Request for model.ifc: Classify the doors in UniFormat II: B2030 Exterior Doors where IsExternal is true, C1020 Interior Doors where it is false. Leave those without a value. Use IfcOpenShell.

First a look at what the model holds.

```python
import ifcopenshell
import ifcopenshell.util.element

model = ifcopenshell.open("model.ifc")
print(model.schema)
print("classifications:", [c.Name for c in model.by_type("IfcClassification")])
values = [ifcopenshell.util.element.get_pset(e, "Pset_DoorCommon", "IsExternal") for e in model.by_type("IfcDoor")]
for value in (True, False, None):
    print("IsExternal", value, values.count(value))
```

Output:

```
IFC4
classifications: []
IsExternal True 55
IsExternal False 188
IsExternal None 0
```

```python
import ifcopenshell
import ifcopenshell.api.classification
import ifcopenshell.util.element

model = ifcopenshell.open("model.ifc")

system = ifcopenshell.api.classification.add_classification(model, classification="UniFormat II")

doors = model.by_type("IfcDoor")
external = {e: ifcopenshell.util.element.get_pset(e, "Pset_DoorCommon", "IsExternal") for e in doors}
for flag, code, name in ((True, "B2030", "Exterior Doors"), (False, "C1020", "Interior Doors")):
    products = [e for e in doors if external[e] is flag]
    ifcopenshell.api.classification.add_reference(
        model, products=products, classification=system, identification=code, name=name
    )
    print(code, len(products))

model.write("model_rev.ifc")
```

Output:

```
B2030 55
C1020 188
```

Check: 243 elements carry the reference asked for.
